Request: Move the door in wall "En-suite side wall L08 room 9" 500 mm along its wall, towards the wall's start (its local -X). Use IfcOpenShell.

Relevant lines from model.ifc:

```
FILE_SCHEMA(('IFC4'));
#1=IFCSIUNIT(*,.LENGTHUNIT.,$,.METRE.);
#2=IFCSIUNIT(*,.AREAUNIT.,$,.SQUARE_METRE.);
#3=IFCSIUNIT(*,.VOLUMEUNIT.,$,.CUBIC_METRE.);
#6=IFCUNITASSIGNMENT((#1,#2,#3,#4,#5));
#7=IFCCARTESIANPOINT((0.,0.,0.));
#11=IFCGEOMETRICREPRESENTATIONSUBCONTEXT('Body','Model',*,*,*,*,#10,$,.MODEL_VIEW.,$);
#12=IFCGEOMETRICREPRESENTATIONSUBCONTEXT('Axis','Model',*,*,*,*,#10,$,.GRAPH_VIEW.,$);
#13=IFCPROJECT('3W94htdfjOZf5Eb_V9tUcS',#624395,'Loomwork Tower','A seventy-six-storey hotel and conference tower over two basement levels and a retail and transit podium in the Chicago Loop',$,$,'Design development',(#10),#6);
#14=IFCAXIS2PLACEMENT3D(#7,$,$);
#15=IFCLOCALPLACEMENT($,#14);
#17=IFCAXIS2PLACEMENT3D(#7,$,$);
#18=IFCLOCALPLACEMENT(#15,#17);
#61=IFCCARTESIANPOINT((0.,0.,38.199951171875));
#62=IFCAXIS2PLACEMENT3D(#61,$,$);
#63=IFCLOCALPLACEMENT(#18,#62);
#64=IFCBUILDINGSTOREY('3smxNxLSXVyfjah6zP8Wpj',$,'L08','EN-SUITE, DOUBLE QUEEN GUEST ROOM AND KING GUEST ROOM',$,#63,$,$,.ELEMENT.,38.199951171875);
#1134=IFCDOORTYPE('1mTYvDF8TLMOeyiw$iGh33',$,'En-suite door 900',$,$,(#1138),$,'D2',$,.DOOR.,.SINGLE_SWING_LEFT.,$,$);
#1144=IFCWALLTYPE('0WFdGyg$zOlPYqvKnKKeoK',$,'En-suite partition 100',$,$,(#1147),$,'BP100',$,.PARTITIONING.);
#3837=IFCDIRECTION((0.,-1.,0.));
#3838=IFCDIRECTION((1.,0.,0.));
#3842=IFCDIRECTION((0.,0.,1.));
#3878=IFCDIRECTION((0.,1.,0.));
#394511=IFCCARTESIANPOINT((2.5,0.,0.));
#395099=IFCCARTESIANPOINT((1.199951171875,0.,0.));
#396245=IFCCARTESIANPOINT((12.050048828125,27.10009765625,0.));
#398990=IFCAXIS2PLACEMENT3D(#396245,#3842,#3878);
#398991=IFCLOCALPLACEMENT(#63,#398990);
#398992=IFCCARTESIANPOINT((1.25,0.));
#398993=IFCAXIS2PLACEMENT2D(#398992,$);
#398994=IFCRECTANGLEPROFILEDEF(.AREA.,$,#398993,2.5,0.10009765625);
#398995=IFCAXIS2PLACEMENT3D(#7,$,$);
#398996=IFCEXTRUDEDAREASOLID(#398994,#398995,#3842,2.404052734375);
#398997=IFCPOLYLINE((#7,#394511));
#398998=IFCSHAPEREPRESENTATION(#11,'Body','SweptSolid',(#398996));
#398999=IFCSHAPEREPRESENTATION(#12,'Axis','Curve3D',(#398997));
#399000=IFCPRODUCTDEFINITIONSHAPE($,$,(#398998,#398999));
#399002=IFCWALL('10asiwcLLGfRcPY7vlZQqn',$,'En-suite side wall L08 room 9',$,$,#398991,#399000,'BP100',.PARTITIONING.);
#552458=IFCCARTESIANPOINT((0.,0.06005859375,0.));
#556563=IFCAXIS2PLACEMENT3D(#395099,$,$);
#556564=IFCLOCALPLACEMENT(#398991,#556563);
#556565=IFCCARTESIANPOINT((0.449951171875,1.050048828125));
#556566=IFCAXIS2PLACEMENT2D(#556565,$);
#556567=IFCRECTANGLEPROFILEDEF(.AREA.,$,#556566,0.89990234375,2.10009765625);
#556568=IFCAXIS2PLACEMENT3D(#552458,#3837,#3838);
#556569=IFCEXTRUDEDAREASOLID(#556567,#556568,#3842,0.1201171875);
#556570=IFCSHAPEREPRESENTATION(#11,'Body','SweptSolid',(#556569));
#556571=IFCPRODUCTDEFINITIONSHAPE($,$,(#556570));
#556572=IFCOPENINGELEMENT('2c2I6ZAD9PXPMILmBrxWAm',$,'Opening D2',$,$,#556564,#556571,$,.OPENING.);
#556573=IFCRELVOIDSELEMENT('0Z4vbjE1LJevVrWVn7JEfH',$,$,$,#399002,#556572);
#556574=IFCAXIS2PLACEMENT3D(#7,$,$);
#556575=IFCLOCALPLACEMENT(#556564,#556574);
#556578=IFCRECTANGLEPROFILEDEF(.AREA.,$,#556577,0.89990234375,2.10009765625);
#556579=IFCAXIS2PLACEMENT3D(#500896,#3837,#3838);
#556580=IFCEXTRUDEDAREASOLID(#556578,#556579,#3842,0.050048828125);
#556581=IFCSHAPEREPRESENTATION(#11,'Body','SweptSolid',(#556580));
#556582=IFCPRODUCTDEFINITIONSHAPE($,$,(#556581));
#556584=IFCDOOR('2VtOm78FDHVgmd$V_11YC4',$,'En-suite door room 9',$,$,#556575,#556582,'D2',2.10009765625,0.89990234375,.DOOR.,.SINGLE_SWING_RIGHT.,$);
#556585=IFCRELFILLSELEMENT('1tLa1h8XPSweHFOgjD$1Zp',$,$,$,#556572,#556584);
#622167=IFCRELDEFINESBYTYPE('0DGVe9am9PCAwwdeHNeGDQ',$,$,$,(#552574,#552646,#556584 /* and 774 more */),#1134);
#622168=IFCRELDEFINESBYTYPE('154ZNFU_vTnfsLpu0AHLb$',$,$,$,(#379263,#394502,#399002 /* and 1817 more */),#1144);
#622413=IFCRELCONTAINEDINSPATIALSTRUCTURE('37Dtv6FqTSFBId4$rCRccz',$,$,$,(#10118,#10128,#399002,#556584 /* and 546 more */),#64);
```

```python
import ifcopenshell
import ifcopenshell.api.geometry
import ifcopenshell.util.placement
import ifcopenshell.util.unit

model = ifcopenshell.open("model.ifc")
unit_scale = ifcopenshell.util.unit.calculate_unit_scale(model)

door = model.by_guid("2VtOm78FDHVgmd$V_11YC4")
opening = door.FillsVoids[0].RelatingOpeningElement
wall = opening.VoidsElements[0].RelatingBuildingElement

wall_matrix = ifcopenshell.util.placement.get_local_placement(wall.ObjectPlacement)
shift = wall_matrix[:3, 0] * -0.5 / unit_scale
before = ifcopenshell.util.placement.get_local_placement(door.ObjectPlacement)[:3, 3].copy()

# The door is placed relative to its opening, so it follows when the opening moves.
matrix = ifcopenshell.util.placement.get_local_placement(opening.ObjectPlacement)
matrix[:3, 3] += shift
ifcopenshell.api.geometry.edit_object_placement(
    model, product=opening, matrix=matrix, is_si=False, should_transform_children=True
)

after = ifcopenshell.util.placement.get_local_placement(door.ObjectPlacement)[:3, 3]
print("door moved by", (after - before).round(3) + 0.0)

model.write("model-out.ifc")
```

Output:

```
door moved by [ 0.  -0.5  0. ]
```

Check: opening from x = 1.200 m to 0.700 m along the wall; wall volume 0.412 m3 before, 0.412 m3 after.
